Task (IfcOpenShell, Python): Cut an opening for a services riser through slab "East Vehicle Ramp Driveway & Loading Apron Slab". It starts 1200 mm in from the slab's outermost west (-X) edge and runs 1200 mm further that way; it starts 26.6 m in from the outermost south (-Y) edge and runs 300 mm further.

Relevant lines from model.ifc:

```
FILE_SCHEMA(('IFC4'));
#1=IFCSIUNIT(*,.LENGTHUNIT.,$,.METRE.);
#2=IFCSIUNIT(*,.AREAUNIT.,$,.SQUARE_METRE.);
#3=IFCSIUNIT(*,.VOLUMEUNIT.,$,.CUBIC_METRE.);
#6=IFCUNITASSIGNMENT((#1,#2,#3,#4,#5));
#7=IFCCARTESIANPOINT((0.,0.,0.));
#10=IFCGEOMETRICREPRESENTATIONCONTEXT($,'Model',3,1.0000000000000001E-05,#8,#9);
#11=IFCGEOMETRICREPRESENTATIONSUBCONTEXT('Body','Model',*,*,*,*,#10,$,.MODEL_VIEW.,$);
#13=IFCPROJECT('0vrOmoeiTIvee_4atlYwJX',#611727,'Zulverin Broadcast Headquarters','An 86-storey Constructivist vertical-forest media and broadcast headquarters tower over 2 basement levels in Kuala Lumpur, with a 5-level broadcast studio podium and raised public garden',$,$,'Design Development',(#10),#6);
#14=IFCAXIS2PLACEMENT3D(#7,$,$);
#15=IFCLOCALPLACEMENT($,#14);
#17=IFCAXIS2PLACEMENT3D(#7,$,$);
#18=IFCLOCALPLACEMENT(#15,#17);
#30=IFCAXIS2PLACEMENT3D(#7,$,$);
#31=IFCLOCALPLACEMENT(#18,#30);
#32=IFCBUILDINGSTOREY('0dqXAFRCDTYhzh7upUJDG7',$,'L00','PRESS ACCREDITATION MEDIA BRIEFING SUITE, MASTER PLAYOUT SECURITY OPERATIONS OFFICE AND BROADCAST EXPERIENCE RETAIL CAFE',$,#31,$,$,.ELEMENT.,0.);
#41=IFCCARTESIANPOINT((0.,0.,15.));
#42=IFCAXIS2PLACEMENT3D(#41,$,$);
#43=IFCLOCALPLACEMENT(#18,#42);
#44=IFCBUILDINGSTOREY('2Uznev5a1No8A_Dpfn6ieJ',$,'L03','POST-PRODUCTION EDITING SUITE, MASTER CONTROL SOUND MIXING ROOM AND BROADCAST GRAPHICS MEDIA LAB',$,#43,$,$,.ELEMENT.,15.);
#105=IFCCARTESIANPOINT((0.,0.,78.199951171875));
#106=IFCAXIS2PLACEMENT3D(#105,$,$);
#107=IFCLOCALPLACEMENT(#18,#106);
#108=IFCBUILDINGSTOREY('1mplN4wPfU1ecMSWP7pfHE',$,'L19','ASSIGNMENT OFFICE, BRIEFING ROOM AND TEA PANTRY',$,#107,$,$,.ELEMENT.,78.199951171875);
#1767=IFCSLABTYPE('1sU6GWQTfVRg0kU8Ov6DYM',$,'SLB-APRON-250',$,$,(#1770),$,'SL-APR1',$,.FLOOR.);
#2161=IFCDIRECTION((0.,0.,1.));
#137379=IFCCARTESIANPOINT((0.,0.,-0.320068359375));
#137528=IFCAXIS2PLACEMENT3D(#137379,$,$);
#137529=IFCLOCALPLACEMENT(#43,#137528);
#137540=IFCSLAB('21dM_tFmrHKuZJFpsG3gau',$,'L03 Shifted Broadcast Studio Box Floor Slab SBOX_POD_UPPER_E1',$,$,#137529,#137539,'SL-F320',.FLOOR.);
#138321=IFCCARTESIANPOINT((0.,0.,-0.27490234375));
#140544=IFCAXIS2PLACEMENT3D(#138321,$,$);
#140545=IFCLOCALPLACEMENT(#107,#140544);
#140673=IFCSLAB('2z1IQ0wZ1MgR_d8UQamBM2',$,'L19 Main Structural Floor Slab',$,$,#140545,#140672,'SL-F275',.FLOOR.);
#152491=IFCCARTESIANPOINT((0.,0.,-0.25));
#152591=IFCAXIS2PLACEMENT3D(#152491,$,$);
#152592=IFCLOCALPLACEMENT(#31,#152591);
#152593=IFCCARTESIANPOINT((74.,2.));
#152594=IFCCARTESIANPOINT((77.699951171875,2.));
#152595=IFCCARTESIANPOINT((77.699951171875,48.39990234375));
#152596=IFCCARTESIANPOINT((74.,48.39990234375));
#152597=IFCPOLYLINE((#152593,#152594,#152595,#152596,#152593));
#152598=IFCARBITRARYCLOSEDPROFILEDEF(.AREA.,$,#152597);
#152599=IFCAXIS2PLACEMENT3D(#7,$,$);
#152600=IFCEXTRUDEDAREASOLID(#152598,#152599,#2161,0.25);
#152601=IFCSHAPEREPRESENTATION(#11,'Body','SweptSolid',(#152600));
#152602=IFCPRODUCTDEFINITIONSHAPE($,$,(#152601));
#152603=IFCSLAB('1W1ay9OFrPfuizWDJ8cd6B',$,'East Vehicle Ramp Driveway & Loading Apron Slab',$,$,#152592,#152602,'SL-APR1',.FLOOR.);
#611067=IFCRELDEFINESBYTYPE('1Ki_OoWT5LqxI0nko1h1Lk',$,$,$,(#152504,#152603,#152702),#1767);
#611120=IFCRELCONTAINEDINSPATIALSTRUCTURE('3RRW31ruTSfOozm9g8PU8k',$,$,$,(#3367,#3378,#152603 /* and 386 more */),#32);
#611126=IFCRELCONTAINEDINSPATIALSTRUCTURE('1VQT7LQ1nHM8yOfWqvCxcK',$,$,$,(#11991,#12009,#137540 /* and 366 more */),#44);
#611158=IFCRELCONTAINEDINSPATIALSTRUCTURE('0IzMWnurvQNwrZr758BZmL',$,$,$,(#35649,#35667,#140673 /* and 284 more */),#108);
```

```python
import numpy as np
import ifcopenshell
import ifcopenshell.api.feature
import ifcopenshell.api.geometry
import ifcopenshell.api.root
import ifcopenshell.geom
import ifcopenshell.util.placement
import ifcopenshell.util.representation
import ifcopenshell.util.shape
import ifcopenshell.util.unit

model = ifcopenshell.open("model.ifc")
unit_scale = ifcopenshell.util.unit.calculate_unit_scale(model)
settings = ifcopenshell.geom.settings()


def volume(element):
    """Net volume in cubic metres, openings subtracted."""
    shape = ifcopenshell.geom.create_shape(settings, element)
    return ifcopenshell.util.shape.get_volume(shape.geometry)


slab = model.by_guid("1W1ay9OFrPfuizWDJ8cd6B")
before = volume(slab)

# Extent in the slab's own axes, in metres. The edges named are its -X and -Y sides.
slab_shape = ifcopenshell.geom.create_shape(settings, slab)
vertices = ifcopenshell.util.shape.get_vertices(slab_shape.geometry)
x_min, y_min, bottom = vertices.min(axis=0)
top = vertices[:, 2].max()

opening = ifcopenshell.api.root.create_entity(model, ifc_class="IfcOpeningElement", name="Services riser opening", predefined_type="OPENING")
context = ifcopenshell.util.representation.get_context(model, "Model", "Body", "MODEL_VIEW")
width, depth = 1.2, 0.3
outline = [(0.0, 0.0), (width, 0.0), (width, depth), (0.0, depth), (0.0, 0.0)]
# Overshoot both faces by 50 mm so the cut is clean.
shape = ifcopenshell.api.geometry.add_slab_representation(
    model, context=context, depth=top - bottom + 0.1, polyline=outline
)
ifcopenshell.api.geometry.assign_representation(model, product=opening, representation=shape)

matrix = ifcopenshell.util.placement.get_local_placement(slab.ObjectPlacement)
matrix[:, 3] = matrix @ np.append(np.array([x_min + 1.2, y_min + 26.6, bottom - 0.05]) / unit_scale, 1.0)
ifcopenshell.api.geometry.edit_object_placement(model, product=opening, matrix=matrix, is_si=False)
ifcopenshell.api.feature.add_feature(model, feature=opening, element=slab)

after = volume(slab)

print(f"slab volume {before:.3f} -> {after:.3f} m3")

model.write("model_updated.ifc")
```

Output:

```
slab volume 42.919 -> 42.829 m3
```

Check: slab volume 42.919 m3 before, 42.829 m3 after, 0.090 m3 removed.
